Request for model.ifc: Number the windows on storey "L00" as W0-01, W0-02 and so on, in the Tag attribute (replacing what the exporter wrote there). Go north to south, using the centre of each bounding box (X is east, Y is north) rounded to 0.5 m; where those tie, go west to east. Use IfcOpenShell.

First a look at what the model holds.

```python
import ifcopenshell
import ifcopenshell.util.element
import ifcopenshell.util.placement

model = ifcopenshell.open("model.ifc")
print(model.schema)
storey = next(s for s in model.by_type("IfcBuildingStorey") if s.Name == "L00")
windows = [e for e in ifcopenshell.util.element.get_decomposition(storey) if e.is_a("IfcWindow")]
for e in sorted(windows, key=lambda e: e.id()):
    origin = ifcopenshell.util.placement.get_local_placement(e.ObjectPlacement)[:3, 3]
    print(e.id(), e.Tag, e.Name, origin.round(2) + 0.0, sep=" | ")
```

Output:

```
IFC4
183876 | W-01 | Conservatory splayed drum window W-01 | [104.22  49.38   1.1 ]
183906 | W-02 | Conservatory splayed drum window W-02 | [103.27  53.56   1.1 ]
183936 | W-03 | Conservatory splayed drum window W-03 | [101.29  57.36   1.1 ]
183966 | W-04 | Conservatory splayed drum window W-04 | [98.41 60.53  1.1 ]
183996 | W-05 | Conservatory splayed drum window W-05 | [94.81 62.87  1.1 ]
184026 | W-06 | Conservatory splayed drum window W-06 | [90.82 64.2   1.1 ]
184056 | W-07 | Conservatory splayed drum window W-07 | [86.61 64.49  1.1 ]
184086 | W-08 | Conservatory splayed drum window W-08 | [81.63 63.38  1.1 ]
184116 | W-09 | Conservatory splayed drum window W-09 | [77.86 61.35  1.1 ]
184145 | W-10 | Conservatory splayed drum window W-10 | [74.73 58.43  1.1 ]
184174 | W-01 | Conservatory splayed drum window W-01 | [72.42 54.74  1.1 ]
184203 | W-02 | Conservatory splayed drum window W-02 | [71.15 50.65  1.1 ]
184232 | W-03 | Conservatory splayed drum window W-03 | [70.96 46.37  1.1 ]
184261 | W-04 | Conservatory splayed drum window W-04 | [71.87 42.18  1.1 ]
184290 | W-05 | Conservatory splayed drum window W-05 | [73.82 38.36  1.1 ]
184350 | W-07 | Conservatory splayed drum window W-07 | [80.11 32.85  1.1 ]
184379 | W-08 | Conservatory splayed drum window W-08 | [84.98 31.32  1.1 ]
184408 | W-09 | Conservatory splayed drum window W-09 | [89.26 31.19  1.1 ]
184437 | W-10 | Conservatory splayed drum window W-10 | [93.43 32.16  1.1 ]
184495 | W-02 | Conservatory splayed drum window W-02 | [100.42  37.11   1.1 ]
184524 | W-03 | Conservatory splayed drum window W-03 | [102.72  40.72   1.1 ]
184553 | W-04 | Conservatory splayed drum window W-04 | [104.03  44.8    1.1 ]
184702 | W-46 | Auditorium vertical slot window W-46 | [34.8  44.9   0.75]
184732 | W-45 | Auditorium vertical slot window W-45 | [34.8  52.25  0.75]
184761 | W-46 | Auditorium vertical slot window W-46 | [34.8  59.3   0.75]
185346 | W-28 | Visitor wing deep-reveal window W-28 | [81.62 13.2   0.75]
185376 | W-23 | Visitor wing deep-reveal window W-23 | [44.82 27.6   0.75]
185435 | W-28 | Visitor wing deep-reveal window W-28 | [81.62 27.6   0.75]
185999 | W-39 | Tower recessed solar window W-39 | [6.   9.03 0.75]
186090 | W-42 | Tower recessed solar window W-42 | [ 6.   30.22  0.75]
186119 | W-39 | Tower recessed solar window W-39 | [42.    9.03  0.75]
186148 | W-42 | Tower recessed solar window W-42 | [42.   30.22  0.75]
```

```python
import ifcopenshell
import ifcopenshell.geom
import ifcopenshell.util.element
import ifcopenshell.util.shape

model = ifcopenshell.open("model.ifc")
settings = ifcopenshell.geom.settings()
settings.set("use-world-coords", True)


def centre(element):
    shape = ifcopenshell.geom.create_shape(settings, element)
    return ifcopenshell.util.shape.get_bbox_centroid(shape.geometry)


storey = next(s for s in model.by_type("IfcBuildingStorey") if s.Name == "L00")
windows = [e for e in ifcopenshell.util.element.get_decomposition(storey) if e.is_a("IfcWindow")]

# Insertion points can sit at a corner or the storey origin, so sort by the geometry (in metres).
centres = {e: centre(e) for e in windows}
windows.sort(key=lambda e: (-round(centres[e][1] / 0.5), centres[e][0]))

for i, e in enumerate(windows, start=1):
    number = f"W0-{i:02d}"
    e.Tag = number
    print(e.id(), number)

model.write("model_rev.ifc")
```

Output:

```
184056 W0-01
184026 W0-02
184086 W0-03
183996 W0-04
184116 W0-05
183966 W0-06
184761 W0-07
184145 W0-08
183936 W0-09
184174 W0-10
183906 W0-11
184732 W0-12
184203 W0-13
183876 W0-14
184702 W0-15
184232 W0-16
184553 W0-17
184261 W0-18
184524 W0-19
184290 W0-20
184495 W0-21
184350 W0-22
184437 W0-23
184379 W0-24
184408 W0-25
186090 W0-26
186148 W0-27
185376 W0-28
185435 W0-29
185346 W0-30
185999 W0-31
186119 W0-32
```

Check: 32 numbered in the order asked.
